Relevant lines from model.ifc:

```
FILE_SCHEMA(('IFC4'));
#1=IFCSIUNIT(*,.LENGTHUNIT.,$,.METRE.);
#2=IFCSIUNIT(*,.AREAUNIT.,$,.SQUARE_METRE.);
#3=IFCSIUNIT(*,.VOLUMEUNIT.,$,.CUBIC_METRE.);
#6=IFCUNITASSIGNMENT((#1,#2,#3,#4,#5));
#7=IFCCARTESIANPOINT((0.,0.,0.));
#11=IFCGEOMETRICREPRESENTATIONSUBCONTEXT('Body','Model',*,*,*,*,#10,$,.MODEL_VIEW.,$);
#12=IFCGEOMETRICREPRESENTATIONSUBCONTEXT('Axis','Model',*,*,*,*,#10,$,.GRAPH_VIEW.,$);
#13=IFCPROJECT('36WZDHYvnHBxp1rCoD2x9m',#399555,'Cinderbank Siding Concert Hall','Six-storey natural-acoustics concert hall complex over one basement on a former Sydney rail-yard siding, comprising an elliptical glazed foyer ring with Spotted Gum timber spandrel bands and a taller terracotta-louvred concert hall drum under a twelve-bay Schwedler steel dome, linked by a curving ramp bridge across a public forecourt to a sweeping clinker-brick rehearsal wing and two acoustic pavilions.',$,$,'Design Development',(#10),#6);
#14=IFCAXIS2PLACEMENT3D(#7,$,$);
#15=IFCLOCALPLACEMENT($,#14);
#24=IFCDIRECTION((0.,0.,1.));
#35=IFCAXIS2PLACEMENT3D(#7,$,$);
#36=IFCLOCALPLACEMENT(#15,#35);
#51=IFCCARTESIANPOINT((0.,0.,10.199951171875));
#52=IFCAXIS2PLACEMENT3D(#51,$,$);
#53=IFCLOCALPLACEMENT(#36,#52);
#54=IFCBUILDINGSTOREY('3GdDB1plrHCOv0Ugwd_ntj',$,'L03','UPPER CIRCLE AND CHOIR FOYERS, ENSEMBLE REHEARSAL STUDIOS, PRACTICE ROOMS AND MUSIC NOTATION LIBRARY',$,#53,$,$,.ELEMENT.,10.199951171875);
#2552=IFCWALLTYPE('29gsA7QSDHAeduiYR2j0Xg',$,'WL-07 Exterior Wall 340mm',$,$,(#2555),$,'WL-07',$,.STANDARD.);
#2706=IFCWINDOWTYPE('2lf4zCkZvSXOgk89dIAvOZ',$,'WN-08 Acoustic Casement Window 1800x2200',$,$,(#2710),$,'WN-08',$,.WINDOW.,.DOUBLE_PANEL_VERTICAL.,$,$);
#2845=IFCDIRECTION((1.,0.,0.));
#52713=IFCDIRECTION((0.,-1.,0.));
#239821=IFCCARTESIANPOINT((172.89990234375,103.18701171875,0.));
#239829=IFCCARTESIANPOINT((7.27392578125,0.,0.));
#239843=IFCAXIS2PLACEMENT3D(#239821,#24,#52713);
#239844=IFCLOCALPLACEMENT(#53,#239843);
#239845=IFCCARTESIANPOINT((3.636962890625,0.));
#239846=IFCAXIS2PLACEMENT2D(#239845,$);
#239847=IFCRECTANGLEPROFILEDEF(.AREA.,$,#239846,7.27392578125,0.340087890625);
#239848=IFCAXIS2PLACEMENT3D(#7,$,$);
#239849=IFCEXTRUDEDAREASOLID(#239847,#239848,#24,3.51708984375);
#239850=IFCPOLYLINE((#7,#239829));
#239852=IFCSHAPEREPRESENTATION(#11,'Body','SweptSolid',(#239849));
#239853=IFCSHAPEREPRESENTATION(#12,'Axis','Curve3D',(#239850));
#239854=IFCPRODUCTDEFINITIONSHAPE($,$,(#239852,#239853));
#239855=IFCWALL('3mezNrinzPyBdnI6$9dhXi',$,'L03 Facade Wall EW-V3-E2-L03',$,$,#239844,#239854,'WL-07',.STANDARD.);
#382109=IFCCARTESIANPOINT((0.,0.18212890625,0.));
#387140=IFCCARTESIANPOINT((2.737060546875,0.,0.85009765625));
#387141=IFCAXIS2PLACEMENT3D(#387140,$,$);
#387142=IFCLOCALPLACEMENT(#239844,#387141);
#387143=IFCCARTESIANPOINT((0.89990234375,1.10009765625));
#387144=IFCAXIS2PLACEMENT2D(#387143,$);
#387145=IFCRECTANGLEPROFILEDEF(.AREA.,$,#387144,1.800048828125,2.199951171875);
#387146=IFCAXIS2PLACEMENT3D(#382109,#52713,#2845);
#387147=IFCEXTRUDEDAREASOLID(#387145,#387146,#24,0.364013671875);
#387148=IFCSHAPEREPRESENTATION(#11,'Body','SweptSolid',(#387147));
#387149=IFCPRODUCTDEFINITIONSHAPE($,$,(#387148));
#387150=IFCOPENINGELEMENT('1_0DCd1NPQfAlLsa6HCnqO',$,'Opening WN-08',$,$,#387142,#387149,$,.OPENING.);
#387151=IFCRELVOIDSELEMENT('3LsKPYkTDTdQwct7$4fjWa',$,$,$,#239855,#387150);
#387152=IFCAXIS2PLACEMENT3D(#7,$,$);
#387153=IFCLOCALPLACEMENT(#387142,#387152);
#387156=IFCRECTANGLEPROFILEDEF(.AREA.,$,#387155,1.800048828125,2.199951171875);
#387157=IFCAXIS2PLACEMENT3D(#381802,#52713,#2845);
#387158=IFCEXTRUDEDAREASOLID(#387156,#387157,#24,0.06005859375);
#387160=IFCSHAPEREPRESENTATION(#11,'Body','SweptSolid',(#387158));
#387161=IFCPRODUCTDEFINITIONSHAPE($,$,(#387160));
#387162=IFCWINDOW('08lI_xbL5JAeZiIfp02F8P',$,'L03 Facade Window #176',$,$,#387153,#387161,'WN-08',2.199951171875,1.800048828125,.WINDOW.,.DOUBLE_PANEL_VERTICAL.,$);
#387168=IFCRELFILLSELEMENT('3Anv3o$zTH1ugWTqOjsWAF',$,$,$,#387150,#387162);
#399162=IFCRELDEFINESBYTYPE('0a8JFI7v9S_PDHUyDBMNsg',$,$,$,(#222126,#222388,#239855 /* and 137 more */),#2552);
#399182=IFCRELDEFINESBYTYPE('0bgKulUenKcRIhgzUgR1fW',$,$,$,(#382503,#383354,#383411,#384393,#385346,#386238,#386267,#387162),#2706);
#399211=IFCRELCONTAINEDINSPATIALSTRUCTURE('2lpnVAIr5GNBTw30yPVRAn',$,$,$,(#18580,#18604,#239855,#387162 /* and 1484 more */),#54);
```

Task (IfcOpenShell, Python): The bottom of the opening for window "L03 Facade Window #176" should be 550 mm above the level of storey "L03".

```python
import numpy as np
import ifcopenshell
import ifcopenshell.api.geometry
import ifcopenshell.geom
import ifcopenshell.util.element
import ifcopenshell.util.placement
import ifcopenshell.util.shape
import ifcopenshell.util.unit

model = ifcopenshell.open("model.ifc")
unit_scale = ifcopenshell.util.unit.calculate_unit_scale(model)

window = model.by_guid("08lI_xbL5JAeZiIfp02F8P")
opening = window.FillsVoids[0].RelatingOpeningElement
storey = ifcopenshell.util.element.get_container(window, ifc_class="IfcBuildingStorey")
level = ifcopenshell.util.placement.get_local_placement(storey.ObjectPlacement)[2, 3]

# The opening's origin need not be at the sill, so measure its lowest point.
shape = ifcopenshell.geom.create_shape(ifcopenshell.geom.settings(), opening)
bottom = ifcopenshell.util.shape.get_shape_bottom_elevation(shape, shape.geometry) / unit_scale
dz = level + 0.55 / unit_scale - bottom

shift = np.array([0.0, 0.0, dz])
# The window is placed relative to its opening, so it follows when the opening moves.
matrix = ifcopenshell.util.placement.get_local_placement(opening.ObjectPlacement)
matrix[:3, 3] += shift
ifcopenshell.api.geometry.edit_object_placement(
    model, product=opening, matrix=matrix, is_si=False, should_transform_children=True
)

print(f"moved by {dz * unit_scale:+.3f} m")

model.write("model_v2.ifc")
```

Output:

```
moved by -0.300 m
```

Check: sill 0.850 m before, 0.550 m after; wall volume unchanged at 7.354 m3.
